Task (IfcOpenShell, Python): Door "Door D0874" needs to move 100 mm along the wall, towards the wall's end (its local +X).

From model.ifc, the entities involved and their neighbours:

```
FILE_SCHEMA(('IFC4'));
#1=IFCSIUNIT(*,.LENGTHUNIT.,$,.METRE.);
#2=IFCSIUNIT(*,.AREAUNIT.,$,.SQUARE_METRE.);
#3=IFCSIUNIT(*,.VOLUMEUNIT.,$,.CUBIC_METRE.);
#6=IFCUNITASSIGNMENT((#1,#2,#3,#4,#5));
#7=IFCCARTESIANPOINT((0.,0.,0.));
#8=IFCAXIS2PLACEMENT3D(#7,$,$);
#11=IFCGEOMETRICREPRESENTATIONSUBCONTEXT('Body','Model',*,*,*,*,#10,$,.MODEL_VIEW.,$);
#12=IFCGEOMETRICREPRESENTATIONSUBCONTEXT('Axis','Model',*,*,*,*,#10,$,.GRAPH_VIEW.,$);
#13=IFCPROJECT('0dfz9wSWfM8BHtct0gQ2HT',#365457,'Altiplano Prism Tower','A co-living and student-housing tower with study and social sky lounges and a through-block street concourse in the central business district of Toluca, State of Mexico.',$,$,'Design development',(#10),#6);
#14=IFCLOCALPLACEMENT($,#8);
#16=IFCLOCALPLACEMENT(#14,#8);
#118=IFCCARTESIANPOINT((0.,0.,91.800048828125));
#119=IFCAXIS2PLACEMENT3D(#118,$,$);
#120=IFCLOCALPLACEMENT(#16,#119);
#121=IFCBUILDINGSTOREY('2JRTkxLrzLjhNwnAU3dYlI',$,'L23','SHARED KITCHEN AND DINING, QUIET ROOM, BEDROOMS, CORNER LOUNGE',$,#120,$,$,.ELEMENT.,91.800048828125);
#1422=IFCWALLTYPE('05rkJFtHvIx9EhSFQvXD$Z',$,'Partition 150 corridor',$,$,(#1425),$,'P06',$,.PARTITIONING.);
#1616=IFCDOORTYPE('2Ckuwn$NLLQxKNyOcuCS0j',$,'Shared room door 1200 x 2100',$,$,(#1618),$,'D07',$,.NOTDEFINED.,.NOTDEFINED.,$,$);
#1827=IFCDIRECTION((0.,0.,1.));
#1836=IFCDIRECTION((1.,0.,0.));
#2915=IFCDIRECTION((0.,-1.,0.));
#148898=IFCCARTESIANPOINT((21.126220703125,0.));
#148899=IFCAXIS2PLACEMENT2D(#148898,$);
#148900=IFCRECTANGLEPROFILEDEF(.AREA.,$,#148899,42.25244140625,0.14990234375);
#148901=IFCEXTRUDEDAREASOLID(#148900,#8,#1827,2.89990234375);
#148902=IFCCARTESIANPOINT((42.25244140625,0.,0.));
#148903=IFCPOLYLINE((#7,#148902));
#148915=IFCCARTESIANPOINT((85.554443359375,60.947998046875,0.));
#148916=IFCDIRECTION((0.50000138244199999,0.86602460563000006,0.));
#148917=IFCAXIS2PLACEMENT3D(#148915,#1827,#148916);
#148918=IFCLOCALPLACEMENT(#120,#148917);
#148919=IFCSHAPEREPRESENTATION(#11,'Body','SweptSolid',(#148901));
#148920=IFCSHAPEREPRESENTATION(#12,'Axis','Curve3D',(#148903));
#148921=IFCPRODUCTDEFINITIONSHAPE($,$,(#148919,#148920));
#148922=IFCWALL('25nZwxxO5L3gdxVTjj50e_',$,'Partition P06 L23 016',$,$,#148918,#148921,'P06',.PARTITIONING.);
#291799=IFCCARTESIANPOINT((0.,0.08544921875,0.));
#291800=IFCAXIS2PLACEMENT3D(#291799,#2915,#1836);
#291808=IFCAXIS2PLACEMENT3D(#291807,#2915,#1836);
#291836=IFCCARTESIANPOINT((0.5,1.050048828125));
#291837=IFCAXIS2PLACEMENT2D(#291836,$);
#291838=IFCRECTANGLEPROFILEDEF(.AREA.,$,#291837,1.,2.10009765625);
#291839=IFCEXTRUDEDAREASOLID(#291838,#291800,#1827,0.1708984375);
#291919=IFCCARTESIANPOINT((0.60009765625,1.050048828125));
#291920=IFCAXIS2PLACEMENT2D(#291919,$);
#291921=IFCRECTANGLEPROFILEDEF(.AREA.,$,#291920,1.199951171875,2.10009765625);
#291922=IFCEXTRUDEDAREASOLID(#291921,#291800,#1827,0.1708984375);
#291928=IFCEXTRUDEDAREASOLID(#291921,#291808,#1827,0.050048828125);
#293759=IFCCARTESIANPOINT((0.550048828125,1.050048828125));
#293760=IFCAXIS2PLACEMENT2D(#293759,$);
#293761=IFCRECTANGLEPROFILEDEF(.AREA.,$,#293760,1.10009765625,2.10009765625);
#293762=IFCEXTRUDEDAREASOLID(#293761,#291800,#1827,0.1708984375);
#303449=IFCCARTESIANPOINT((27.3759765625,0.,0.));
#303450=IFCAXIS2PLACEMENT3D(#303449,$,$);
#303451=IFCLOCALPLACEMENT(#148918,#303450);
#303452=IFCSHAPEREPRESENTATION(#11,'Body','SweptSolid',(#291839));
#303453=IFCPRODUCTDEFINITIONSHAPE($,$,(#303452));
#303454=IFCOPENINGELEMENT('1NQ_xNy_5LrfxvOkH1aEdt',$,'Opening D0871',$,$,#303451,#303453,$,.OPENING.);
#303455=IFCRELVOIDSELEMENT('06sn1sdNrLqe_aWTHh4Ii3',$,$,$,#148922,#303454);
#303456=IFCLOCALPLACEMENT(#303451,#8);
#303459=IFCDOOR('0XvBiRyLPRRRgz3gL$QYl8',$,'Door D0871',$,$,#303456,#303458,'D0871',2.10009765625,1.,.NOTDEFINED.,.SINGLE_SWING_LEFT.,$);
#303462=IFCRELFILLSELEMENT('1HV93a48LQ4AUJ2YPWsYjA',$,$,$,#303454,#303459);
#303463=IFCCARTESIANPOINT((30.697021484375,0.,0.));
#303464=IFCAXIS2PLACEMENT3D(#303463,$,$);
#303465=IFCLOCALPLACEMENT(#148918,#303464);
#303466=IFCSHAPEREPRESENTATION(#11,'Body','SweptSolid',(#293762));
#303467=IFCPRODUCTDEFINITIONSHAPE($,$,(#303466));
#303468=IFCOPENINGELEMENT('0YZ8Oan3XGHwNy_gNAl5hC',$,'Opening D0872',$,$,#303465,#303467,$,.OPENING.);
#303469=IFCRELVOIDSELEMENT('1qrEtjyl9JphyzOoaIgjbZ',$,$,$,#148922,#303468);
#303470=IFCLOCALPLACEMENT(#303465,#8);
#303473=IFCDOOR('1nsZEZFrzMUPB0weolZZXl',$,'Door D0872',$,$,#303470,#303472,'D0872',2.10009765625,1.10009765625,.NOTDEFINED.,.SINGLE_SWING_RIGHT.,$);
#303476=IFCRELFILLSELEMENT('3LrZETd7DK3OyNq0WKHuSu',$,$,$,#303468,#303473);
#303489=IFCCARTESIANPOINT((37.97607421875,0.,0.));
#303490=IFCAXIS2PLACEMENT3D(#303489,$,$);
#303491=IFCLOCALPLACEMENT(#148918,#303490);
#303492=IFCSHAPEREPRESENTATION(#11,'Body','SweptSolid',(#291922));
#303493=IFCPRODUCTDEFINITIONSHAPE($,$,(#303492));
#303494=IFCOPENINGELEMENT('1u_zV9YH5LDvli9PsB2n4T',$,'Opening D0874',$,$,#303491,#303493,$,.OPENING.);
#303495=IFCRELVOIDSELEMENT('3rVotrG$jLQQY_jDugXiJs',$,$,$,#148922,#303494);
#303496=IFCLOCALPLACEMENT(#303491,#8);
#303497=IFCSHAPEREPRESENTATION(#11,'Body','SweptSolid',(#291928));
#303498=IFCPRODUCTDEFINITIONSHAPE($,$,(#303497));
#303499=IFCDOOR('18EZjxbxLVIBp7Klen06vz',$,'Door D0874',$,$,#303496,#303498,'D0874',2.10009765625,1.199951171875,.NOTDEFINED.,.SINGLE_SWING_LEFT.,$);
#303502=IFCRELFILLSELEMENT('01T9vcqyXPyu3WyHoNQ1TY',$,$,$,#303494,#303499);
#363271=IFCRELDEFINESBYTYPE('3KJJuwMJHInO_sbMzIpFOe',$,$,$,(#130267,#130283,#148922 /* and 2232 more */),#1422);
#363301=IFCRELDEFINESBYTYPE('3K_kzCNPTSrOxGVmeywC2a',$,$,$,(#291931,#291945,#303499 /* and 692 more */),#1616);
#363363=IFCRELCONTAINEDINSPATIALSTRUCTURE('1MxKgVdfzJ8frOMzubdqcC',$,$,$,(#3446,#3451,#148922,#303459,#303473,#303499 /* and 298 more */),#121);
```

```python
import ifcopenshell
import ifcopenshell.api.geometry
import ifcopenshell.util.placement

model = ifcopenshell.open("model.ifc")

door = model.by_id(303499)
opening = door.FillsVoids[0].RelatingOpeningElement
wall = opening.VoidsElements[0].RelatingBuildingElement

wall_matrix = ifcopenshell.util.placement.get_local_placement(wall.ObjectPlacement)
shift = wall_matrix[:3, 0] * 0.1
before = ifcopenshell.util.placement.get_local_placement(door.ObjectPlacement)[:3, 3].copy()

# The door is placed relative to its opening, so it follows when the opening moves.
matrix = ifcopenshell.util.placement.get_local_placement(opening.ObjectPlacement)
matrix[:3, 3] += shift
ifcopenshell.api.geometry.edit_object_placement(
    model, product=opening, matrix=matrix, is_si=False, should_transform_children=True
)

after = ifcopenshell.util.placement.get_local_placement(door.ObjectPlacement)[:3, 3]
print("door moved by", (after - before).round(3) + 0.0)

model.write("model_updated.ifc")
```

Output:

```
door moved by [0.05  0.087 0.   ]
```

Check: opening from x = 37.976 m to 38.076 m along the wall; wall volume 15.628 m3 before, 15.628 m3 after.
